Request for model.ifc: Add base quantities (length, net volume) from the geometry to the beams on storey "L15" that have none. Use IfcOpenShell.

First a look at what the model holds.

```python
import ifcopenshell
import ifcopenshell.util.element
import ifcopenshell.util.unit

model = ifcopenshell.open("model.ifc")
print(model.schema)
for unit_type in ("LENGTHUNIT", "AREAUNIT", "VOLUMEUNIT"):
    print(unit_type, ifcopenshell.util.unit.calculate_unit_scale(model, unit_type))
storey = next(s for s in model.by_type("IfcBuildingStorey") if s.Name == "L15")
beams = [e for e in ifcopenshell.util.element.get_decomposition(storey) if e.is_a("IfcBeam")]
for e in sorted(beams, key=lambda e: e.id()):
    print(e.id(), e.is_a(), e.Name, list(ifcopenshell.util.element.get_psets(e, qtos_only=True)), sep=" | ")
```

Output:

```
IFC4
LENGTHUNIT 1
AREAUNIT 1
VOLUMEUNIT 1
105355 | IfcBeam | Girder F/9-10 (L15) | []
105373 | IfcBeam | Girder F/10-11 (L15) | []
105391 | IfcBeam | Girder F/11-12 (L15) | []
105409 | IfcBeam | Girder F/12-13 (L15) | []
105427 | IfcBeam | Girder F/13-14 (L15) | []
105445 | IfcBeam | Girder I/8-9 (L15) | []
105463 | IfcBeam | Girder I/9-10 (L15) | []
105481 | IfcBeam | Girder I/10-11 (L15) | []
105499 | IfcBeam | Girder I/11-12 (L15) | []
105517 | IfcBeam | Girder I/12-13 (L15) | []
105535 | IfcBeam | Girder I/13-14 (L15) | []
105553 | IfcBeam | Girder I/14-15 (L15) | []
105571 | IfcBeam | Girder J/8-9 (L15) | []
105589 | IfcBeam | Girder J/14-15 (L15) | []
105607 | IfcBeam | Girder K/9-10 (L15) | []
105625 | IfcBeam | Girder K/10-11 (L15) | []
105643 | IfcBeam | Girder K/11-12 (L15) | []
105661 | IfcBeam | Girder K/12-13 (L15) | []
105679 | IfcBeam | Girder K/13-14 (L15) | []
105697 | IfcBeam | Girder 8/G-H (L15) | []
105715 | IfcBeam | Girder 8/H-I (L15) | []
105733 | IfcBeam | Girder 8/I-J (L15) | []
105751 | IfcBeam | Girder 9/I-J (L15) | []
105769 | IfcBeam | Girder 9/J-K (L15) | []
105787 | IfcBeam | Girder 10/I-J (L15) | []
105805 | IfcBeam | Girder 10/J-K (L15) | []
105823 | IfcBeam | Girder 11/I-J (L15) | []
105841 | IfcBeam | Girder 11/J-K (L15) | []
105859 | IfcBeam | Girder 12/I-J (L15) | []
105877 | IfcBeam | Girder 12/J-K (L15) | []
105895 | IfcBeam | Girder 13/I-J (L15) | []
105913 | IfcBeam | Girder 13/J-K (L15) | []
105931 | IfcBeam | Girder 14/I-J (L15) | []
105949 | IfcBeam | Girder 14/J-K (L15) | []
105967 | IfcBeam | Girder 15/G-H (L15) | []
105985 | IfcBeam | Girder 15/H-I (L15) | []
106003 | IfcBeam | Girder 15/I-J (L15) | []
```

```python
import ifcopenshell
import ifcopenshell.api.pset
import ifcopenshell.geom
import ifcopenshell.util.element
import ifcopenshell.util.shape
import ifcopenshell.util.unit

model = ifcopenshell.open("model.ifc")
unit_scale = ifcopenshell.util.unit.calculate_unit_scale(model)
volume_scale = ifcopenshell.util.unit.calculate_unit_scale(model, "VOLUMEUNIT")
settings = ifcopenshell.geom.settings()

storey = next(s for s in model.by_type("IfcBuildingStorey") if s.Name == "L15")
beams = [e for e in ifcopenshell.util.element.get_decomposition(storey) if e.is_a("IfcBeam")]

for e in sorted(beams, key=lambda e: e.id()):
    if ifcopenshell.util.element.get_psets(e, qtos_only=True, should_inherit=False):
        continue
    # Geometry comes back in metres, in the element's own axes.
    shape = ifcopenshell.geom.create_shape(settings, e)
    values = {
        "Length": ifcopenshell.util.shape.get_max_xyz(shape.geometry) / unit_scale,
        "NetVolume": ifcopenshell.util.shape.get_volume(shape.geometry) / volume_scale,
    }
    qto = ifcopenshell.api.pset.add_qto(model, product=e, name="Qto_BeamBaseQuantities")
    ifcopenshell.api.pset.edit_qto(model, qto=qto, properties=values)
    print(e.id(), {k: round(v, 3) for k, v in values.items()})

model.write("model_edited.ifc")
```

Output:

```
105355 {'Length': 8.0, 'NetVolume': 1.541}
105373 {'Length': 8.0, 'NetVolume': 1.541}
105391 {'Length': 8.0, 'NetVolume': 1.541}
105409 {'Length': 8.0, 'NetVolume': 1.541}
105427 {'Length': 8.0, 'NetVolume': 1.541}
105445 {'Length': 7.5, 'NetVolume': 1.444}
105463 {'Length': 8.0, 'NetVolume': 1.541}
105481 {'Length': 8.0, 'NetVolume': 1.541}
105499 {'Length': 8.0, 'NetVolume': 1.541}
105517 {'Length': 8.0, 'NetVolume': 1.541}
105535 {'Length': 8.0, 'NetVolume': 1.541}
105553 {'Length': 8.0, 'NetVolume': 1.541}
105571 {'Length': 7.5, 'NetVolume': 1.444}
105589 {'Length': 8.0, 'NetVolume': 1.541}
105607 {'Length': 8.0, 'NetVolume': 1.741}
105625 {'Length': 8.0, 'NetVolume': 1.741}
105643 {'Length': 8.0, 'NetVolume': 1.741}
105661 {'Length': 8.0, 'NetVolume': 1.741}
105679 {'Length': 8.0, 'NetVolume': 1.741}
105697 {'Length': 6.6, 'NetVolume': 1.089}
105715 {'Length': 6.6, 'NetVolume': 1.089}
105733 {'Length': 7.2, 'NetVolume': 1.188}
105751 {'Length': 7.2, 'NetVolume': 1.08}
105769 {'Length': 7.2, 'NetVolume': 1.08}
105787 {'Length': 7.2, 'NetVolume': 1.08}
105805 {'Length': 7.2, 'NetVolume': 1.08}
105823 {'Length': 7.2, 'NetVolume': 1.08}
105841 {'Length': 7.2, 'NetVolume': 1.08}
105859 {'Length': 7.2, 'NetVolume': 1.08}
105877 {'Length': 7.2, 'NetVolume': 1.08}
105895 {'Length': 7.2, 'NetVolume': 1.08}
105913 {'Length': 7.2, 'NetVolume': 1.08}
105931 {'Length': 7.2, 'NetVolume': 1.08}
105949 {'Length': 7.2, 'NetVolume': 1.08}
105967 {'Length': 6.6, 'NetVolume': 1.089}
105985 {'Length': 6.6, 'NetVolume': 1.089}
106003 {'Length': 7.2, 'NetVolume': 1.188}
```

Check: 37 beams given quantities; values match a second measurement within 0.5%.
